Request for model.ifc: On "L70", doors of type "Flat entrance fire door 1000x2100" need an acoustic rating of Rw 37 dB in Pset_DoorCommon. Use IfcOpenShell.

First a look at what the model holds.

```python
import ifcopenshell
import ifcopenshell.util.element

model = ifcopenshell.open("model.ifc")
print(model.schema)
storey = next(s for s in model.by_type("IfcBuildingStorey") if s.Name == "L70")
doors = [e for e in ifcopenshell.util.element.get_decomposition(storey) if e.is_a("IfcDoor")]
seen = {}
for e in doors:
    element_type = ifcopenshell.util.element.get_type(e)
    key = (element_type.Name if element_type != e and element_type else None, ifcopenshell.util.element.get_pset(e, "Pset_DoorCommon", "AcousticRating"))
    seen[key] = seen.get(key, 0) + 1
for (name, value), count in sorted(seen.items(), key=str):
    print(count, "x", name, "|", value)
```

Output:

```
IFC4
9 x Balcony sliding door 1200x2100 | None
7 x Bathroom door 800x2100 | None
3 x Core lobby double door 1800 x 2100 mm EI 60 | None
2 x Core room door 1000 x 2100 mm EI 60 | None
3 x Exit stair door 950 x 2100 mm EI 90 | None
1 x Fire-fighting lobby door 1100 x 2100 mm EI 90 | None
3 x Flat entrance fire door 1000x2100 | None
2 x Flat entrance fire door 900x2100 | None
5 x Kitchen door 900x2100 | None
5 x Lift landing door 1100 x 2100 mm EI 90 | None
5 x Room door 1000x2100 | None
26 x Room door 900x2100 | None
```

```python
import ifcopenshell
import ifcopenshell.api.pset
import ifcopenshell.util.element

model = ifcopenshell.open("model.ifc")

storey = next(s for s in model.by_type("IfcBuildingStorey") if s.Name == "L70")
doors = [e for e in ifcopenshell.util.element.get_decomposition(storey) if e.is_a("IfcDoor")]

count = 0
for e in doors:
    element_type = ifcopenshell.util.element.get_type(e)
    if element_type in (None, e) or element_type.Name != "Flat entrance fire door 1000x2100":
        continue
    found = ifcopenshell.util.element.get_pset(e, "Pset_DoorCommon", should_inherit=False)
    if found:
        pset = model.by_id(found["id"])
        if len(ifcopenshell.util.element.get_elements_by_pset(pset)) > 1:
            pset = ifcopenshell.api.pset.unshare_pset(model, products=[e], pset=pset)[0]
    else:
        pset = ifcopenshell.api.pset.add_pset(model, product=e, name="Pset_DoorCommon")
    ifcopenshell.api.pset.edit_pset(model, pset=pset, properties={"AcousticRating": "Rw 37 dB"})
    count += 1

print(count, "doors updated")

model.write("model_v2.ifc")
```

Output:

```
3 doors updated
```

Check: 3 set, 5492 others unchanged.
